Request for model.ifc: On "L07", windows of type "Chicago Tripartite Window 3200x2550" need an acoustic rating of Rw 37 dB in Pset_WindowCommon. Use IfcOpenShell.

First a look at what the model holds.

```python
import ifcopenshell
import ifcopenshell.util.element

model = ifcopenshell.open("model.ifc")
print(model.schema)
storey = next(s for s in model.by_type("IfcBuildingStorey") if s.Name == "L07")
windows = [e for e in ifcopenshell.util.element.get_decomposition(storey) if e.is_a("IfcWindow")]
seen = {}
for e in windows:
    element_type = ifcopenshell.util.element.get_type(e)
    key = (element_type.Name if element_type != e and element_type else None, ifcopenshell.util.element.get_pset(e, "Pset_WindowCommon", "AcousticRating"))
    seen[key] = seen.get(key, 0) + 1
for (name, value), count in sorted(seen.items(), key=str):
    print(count, "x", name, "|", value)
```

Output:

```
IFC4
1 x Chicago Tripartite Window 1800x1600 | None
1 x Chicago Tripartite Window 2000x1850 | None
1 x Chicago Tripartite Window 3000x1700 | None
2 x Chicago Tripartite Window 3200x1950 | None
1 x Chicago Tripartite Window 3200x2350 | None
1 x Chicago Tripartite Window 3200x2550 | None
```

```python
import ifcopenshell
import ifcopenshell.api.pset
import ifcopenshell.util.element

model = ifcopenshell.open("model.ifc")

storey = next(s for s in model.by_type("IfcBuildingStorey") if s.Name == "L07")
windows = [e for e in ifcopenshell.util.element.get_decomposition(storey) if e.is_a("IfcWindow")]

count = 0
for e in windows:
    element_type = ifcopenshell.util.element.get_type(e)
    if element_type in (None, e) or element_type.Name != "Chicago Tripartite Window 3200x2550":
        continue
    # add_pset returns the element's existing set when there is one.
    pset = ifcopenshell.api.pset.add_pset(model, product=e, name="Pset_WindowCommon")
    ifcopenshell.api.pset.edit_pset(model, pset=pset, properties={"AcousticRating": "Rw 37 dB"})
    count += 1

print(count, "windows updated")

model.write("model_rev.ifc")
```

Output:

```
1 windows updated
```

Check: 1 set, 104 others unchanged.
